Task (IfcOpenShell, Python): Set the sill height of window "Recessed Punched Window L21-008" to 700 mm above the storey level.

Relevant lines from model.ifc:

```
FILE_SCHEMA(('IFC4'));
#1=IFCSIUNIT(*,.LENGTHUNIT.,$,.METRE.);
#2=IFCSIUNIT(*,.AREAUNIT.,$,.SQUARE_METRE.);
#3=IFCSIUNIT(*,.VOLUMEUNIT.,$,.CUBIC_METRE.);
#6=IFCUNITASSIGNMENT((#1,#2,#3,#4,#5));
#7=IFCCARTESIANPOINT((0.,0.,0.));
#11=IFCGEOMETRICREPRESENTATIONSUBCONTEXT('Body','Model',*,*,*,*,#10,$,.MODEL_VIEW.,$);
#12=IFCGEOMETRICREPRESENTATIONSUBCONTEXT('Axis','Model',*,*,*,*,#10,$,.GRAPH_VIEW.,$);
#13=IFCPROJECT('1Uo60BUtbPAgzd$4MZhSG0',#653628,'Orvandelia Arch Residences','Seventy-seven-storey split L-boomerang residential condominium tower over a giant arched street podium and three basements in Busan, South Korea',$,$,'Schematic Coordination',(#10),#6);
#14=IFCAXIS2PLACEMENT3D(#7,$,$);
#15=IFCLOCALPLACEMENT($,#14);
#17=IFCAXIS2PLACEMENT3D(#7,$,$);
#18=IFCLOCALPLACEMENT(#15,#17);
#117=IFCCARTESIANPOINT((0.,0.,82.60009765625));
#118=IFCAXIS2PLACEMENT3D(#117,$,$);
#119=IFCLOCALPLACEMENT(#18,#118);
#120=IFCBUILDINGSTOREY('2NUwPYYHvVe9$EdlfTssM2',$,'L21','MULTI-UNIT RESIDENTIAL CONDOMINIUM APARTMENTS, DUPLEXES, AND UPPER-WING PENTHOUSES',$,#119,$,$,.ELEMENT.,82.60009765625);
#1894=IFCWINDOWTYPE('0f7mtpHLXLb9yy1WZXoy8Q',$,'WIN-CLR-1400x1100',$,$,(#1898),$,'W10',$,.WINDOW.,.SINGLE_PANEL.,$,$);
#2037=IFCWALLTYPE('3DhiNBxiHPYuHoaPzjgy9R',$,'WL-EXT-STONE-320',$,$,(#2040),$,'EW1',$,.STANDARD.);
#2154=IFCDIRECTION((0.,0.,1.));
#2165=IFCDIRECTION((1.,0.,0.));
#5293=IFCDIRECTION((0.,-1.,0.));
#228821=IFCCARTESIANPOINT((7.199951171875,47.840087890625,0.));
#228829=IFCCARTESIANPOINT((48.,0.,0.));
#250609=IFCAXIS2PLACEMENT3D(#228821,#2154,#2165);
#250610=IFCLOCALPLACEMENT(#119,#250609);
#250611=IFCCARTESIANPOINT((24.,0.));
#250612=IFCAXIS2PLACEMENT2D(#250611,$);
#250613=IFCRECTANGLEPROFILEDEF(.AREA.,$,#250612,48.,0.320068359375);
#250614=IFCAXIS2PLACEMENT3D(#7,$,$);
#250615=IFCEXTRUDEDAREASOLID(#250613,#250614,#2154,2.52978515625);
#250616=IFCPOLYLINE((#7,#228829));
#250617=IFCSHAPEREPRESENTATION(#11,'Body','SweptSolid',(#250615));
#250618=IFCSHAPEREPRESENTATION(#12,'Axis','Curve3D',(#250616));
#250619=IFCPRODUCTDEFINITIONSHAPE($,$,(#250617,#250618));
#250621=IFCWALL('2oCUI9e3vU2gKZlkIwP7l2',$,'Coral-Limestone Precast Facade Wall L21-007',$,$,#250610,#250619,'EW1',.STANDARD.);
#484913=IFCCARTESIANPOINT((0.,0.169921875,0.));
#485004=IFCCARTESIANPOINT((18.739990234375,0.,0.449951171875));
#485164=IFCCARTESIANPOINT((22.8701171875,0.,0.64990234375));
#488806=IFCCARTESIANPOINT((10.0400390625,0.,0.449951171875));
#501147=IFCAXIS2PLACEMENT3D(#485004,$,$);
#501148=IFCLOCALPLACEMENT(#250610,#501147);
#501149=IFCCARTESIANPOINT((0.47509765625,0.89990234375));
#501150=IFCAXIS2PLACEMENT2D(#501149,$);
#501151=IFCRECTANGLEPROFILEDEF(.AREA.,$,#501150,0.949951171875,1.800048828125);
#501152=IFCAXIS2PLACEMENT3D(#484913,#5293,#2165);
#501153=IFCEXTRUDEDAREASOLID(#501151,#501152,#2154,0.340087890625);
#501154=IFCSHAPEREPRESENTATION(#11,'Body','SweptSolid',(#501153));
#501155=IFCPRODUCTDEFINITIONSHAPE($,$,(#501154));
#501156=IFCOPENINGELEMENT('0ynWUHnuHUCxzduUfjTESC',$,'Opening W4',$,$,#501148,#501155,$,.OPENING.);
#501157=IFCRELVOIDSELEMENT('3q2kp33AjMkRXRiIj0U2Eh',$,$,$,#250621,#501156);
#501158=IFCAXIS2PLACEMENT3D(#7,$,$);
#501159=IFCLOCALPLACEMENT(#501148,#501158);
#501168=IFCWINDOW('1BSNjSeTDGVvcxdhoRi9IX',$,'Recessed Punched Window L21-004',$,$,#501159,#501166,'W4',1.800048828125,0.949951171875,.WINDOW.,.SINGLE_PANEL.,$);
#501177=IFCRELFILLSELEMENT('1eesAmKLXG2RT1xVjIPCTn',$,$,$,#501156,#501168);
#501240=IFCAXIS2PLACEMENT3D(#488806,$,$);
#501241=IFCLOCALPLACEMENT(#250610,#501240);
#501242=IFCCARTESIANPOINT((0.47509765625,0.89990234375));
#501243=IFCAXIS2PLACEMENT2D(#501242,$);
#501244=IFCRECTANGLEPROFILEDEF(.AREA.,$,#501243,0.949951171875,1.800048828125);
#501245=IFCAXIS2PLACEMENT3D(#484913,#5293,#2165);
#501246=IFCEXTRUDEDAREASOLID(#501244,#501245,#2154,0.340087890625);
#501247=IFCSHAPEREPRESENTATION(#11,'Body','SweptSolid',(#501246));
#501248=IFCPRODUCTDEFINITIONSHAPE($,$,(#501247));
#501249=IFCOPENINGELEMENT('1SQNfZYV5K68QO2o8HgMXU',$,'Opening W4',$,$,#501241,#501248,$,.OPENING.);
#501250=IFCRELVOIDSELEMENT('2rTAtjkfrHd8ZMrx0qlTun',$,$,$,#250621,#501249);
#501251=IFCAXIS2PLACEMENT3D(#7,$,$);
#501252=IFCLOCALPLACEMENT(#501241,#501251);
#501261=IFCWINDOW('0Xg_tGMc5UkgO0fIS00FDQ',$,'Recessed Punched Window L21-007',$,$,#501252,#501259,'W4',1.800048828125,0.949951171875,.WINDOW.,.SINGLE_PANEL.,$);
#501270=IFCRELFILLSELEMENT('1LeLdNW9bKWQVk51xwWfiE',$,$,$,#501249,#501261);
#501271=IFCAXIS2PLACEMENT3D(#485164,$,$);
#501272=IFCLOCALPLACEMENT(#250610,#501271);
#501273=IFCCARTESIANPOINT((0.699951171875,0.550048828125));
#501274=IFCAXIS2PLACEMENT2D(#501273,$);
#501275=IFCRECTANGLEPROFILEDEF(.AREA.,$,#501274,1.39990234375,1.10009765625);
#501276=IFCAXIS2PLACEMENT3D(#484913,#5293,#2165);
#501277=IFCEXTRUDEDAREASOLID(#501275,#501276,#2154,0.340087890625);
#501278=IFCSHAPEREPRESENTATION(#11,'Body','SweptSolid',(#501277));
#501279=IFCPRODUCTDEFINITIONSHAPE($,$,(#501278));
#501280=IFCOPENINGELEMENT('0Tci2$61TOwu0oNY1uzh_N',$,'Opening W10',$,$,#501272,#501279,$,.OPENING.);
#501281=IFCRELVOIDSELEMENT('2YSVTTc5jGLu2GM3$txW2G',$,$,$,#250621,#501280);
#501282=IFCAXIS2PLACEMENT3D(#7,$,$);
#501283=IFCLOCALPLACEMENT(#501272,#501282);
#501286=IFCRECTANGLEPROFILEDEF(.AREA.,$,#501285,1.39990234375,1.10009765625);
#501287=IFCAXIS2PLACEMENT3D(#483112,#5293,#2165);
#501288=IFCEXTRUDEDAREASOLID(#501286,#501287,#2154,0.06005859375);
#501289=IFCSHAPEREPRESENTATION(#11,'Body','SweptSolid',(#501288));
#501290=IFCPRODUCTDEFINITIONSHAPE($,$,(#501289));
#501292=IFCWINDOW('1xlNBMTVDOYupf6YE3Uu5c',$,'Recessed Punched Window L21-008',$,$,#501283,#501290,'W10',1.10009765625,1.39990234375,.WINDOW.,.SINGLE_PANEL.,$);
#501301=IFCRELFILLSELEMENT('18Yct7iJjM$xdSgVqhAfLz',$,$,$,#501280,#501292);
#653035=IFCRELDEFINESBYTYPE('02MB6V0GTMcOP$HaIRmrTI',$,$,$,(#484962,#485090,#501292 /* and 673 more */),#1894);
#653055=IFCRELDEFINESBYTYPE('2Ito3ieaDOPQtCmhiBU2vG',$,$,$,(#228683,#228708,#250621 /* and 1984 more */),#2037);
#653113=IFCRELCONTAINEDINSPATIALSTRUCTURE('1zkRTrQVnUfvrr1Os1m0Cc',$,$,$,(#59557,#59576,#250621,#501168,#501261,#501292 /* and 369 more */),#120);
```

```python
import numpy as np
import ifcopenshell
import ifcopenshell.api.geometry
import ifcopenshell.geom
import ifcopenshell.util.element
import ifcopenshell.util.placement
import ifcopenshell.util.shape
import ifcopenshell.util.unit

model = ifcopenshell.open("model.ifc")
unit_scale = ifcopenshell.util.unit.calculate_unit_scale(model)

window = model.by_guid("1xlNBMTVDOYupf6YE3Uu5c")
opening = window.FillsVoids[0].RelatingOpeningElement
storey = ifcopenshell.util.element.get_container(window, ifc_class="IfcBuildingStorey")
level = ifcopenshell.util.placement.get_local_placement(storey.ObjectPlacement)[2, 3]

# The opening's origin need not be at the sill, so measure its lowest point.
shape = ifcopenshell.geom.create_shape(ifcopenshell.geom.settings(), opening)
bottom = ifcopenshell.util.shape.get_shape_bottom_elevation(shape, shape.geometry) / unit_scale
dz = level + 0.7 - bottom

shift = np.array([0.0, 0.0, dz])
# The window is placed relative to its opening, so it follows when the opening moves.
matrix = ifcopenshell.util.placement.get_local_placement(opening.ObjectPlacement)
matrix[:3, 3] += shift
ifcopenshell.api.geometry.edit_object_placement(
    model, product=opening, matrix=matrix, is_si=False, should_transform_children=True
)

print(f"moved by {dz * unit_scale:+.3f} m")

model.write("model-out.ifc")
```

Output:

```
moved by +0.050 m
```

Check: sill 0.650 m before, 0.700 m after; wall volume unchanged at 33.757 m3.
